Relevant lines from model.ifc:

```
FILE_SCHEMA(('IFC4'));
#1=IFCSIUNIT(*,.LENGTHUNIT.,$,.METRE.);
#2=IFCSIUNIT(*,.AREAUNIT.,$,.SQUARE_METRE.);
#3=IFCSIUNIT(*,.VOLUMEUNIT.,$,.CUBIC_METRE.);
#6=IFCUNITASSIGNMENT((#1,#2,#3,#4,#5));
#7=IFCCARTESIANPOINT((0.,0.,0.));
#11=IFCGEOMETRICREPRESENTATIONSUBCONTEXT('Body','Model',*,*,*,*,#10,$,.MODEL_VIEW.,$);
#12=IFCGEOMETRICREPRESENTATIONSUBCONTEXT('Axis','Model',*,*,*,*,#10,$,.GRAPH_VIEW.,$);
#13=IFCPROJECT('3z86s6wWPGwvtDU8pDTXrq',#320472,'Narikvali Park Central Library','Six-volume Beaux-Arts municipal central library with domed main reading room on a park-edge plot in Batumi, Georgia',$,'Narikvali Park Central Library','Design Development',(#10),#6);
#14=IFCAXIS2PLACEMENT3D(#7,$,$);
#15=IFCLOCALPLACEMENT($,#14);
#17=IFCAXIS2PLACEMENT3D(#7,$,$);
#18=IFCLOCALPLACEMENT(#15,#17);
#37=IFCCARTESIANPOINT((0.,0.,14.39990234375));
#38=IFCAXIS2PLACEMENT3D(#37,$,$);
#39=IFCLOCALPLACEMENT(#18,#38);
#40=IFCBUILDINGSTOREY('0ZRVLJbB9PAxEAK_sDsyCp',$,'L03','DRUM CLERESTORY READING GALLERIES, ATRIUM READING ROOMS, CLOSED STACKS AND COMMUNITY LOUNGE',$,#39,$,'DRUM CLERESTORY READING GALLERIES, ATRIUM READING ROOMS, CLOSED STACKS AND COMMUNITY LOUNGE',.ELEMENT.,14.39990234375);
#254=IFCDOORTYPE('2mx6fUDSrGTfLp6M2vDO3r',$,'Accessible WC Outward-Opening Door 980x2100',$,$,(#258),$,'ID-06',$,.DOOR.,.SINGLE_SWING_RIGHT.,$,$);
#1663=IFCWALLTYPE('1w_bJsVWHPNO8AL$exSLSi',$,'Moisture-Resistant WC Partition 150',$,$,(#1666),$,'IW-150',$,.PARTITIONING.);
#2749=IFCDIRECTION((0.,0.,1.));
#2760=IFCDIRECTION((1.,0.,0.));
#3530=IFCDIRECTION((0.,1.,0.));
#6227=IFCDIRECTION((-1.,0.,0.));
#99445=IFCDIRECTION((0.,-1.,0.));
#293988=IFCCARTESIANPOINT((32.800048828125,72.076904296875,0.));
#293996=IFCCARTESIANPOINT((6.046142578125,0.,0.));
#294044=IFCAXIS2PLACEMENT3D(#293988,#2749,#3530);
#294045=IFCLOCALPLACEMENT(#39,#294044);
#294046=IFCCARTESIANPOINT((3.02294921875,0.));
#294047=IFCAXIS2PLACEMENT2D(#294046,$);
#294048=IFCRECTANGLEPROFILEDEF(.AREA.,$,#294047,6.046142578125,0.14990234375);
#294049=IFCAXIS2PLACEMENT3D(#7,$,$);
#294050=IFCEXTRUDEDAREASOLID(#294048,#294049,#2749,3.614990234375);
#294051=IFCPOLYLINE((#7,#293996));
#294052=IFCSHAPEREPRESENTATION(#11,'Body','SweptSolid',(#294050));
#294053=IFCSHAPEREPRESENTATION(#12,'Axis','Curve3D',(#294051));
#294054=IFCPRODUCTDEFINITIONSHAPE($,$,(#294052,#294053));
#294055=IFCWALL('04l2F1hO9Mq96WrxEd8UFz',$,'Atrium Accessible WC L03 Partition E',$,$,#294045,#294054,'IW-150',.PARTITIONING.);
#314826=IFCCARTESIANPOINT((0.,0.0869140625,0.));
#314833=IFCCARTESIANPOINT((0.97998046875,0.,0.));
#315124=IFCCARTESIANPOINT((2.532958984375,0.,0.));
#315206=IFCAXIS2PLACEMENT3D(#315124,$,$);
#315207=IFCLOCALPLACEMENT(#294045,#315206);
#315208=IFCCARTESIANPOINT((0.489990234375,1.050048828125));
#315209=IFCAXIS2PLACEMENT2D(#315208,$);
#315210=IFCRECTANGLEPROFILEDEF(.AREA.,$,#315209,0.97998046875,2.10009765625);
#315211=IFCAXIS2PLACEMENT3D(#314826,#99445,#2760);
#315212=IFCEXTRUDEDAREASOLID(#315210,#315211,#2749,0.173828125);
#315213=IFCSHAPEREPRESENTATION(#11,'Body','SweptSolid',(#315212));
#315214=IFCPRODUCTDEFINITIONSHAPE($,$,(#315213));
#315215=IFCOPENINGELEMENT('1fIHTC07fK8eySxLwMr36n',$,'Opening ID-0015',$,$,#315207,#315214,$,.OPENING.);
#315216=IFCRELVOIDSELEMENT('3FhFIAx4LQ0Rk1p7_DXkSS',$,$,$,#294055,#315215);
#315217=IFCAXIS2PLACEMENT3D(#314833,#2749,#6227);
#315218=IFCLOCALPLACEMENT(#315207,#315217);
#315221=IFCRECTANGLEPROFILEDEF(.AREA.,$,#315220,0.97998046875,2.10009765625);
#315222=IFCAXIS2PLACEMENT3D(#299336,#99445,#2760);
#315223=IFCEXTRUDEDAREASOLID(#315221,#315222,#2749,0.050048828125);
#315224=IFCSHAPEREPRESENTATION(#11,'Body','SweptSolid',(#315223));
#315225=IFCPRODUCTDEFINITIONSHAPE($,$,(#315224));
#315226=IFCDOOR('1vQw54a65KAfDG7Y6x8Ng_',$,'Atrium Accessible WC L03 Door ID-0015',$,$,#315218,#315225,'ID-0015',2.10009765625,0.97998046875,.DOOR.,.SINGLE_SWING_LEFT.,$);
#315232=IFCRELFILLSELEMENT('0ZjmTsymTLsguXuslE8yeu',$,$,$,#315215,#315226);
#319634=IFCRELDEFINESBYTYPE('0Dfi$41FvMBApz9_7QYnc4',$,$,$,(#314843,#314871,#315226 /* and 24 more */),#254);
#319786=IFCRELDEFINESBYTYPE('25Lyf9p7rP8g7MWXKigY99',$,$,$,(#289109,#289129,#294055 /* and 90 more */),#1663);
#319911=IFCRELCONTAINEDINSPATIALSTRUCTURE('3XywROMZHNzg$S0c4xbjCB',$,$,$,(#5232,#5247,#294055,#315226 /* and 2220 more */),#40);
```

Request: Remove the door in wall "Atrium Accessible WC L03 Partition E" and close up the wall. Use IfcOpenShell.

```python
import ifcopenshell
import ifcopenshell.api.feature
import ifcopenshell.api.root
import ifcopenshell.geom
import ifcopenshell.util.shape

model = ifcopenshell.open("model.ifc")
settings = ifcopenshell.geom.settings()


def volume(element):
    """Net volume in cubic metres, openings subtracted."""
    shape = ifcopenshell.geom.create_shape(settings, element)
    return ifcopenshell.util.shape.get_volume(shape.geometry)


door = model.by_guid("1vQw54a65KAfDG7Y6x8Ng_")
opening = door.FillsVoids[0].RelatingOpeningElement
wall = opening.VoidsElements[0].RelatingBuildingElement
before = volume(wall)

ifcopenshell.api.root.remove_product(model, product=door)
ifcopenshell.api.feature.remove_feature(model, feature=opening)

after = volume(wall)

print(f"wall volume {before:.3f} -> {after:.3f} m3")

model.write("model_edited.ifc")
```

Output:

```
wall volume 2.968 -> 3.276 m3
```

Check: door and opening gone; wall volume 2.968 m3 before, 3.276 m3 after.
